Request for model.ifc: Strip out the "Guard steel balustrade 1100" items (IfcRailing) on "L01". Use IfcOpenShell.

First a look at what the model holds.

```python
import ifcopenshell
import ifcopenshell.util.element

model = ifcopenshell.open("model.ifc")
print(model.schema)
storey = next(s for s in model.by_type("IfcBuildingStorey") if s.Name == "L01")
railings = [e for e in ifcopenshell.util.element.get_decomposition(storey) if e.is_a("IfcRailing")]
seen = {}
for e in railings:
    element_type = ifcopenshell.util.element.get_type(e)
    name = element_type.Name if element_type not in (None, e) else None
    seen[name] = seen.get(name, 0) + 1
for name, count in sorted(seen.items(), key=str):
    print(count, "x", name)
```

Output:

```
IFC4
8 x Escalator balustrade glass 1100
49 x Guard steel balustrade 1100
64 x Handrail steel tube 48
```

```python
import ifcopenshell
import ifcopenshell.api.root
import ifcopenshell.util.element

model = ifcopenshell.open("model.ifc")

storey = next(s for s in model.by_type("IfcBuildingStorey") if s.Name == "L01")
railings = [e for e in ifcopenshell.util.element.get_decomposition(storey) if e.is_a("IfcRailing")]
targets = [e for e in railings if (t := ifcopenshell.util.element.get_type(e)) not in (None, e) and t.Name == "Guard steel balustrade 1100"]

for e in targets:
    ifcopenshell.api.root.remove_product(model, product=e)
print(len(targets), "removed")

model.write("model_edited.ifc")
```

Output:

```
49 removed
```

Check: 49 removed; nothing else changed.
